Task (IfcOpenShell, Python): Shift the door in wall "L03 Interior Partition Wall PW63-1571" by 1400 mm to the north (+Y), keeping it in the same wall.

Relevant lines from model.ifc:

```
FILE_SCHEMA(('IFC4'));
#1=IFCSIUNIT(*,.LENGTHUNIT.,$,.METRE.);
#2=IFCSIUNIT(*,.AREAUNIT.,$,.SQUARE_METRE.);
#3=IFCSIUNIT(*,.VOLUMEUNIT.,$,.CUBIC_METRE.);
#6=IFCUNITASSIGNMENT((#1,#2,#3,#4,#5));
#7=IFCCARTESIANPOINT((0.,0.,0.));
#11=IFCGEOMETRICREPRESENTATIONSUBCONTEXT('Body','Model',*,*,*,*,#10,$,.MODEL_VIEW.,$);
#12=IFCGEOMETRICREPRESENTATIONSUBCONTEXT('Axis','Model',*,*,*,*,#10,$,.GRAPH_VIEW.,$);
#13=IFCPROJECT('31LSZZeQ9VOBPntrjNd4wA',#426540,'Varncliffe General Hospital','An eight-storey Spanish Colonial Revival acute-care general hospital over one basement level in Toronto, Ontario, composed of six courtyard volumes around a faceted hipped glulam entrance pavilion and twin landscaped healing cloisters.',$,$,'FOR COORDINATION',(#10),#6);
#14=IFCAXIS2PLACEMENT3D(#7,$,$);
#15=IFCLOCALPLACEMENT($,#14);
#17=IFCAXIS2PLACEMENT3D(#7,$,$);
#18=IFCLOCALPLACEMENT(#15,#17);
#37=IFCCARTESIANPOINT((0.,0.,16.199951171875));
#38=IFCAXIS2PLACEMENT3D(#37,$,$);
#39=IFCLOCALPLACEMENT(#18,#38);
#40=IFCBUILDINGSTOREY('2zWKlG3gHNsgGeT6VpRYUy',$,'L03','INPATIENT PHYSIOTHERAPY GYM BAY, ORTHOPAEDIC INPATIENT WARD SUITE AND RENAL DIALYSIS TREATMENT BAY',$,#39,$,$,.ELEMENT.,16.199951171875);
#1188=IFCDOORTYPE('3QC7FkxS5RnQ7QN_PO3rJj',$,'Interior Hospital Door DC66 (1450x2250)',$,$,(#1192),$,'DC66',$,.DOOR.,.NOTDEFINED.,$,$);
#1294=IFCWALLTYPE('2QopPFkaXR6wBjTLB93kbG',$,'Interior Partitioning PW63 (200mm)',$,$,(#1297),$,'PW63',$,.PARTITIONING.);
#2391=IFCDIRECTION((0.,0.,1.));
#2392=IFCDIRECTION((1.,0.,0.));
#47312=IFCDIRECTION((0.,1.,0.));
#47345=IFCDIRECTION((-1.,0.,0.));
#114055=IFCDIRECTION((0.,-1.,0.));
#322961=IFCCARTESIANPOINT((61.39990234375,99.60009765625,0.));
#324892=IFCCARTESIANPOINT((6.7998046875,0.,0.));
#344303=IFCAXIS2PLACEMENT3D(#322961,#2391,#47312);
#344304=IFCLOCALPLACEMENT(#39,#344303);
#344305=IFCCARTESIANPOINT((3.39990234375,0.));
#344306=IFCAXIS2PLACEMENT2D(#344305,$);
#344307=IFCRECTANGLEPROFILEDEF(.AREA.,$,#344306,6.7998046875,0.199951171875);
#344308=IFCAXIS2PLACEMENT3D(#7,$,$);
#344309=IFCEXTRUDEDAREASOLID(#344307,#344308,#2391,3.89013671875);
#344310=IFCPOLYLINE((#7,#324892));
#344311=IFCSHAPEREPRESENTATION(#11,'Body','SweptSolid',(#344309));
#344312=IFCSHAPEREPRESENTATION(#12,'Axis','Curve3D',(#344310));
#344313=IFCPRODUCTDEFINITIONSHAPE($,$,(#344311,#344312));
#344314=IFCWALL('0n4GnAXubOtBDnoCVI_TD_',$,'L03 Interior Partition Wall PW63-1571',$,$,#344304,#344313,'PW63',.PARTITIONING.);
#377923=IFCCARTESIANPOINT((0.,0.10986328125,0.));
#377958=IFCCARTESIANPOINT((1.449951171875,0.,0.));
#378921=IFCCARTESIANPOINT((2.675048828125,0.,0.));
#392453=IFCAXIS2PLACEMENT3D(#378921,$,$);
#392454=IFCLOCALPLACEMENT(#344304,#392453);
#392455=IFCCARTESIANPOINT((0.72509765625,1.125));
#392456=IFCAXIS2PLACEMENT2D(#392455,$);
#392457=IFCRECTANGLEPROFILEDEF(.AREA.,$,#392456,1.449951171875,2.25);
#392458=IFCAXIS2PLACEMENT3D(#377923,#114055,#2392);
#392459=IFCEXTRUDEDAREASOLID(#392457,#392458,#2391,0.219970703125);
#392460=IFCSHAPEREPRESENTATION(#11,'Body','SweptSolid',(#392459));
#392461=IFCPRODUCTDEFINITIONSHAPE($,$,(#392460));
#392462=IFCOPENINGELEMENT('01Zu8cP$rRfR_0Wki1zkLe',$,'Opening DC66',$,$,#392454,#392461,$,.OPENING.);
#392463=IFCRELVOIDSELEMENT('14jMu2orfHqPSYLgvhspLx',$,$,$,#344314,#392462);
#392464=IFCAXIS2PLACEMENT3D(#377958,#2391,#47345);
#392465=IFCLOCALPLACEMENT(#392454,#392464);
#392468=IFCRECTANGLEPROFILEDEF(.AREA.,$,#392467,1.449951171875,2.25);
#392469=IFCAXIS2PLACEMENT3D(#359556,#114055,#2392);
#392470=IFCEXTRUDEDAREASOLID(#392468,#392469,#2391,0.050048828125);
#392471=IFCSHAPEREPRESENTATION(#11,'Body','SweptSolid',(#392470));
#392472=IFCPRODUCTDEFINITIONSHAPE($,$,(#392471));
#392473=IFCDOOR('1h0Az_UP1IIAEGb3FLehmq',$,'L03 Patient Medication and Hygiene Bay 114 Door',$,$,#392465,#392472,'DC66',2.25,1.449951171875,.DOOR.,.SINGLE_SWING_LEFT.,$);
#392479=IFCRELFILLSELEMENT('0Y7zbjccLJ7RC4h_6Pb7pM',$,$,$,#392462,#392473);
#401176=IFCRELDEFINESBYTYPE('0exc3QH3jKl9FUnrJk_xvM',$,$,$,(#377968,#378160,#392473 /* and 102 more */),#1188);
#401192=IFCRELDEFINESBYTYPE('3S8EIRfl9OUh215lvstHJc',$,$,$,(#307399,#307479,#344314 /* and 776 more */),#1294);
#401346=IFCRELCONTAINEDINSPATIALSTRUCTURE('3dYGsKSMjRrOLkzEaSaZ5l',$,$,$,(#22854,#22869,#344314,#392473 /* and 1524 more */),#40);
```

```python
import ifcopenshell
import ifcopenshell.api.geometry
import ifcopenshell.util.placement
import ifcopenshell.util.unit

model = ifcopenshell.open("model.ifc")
unit_scale = ifcopenshell.util.unit.calculate_unit_scale(model)

door = model.by_guid("1h0Az_UP1IIAEGb3FLehmq")
opening = door.FillsVoids[0].RelatingOpeningElement
wall = opening.VoidsElements[0].RelatingBuildingElement

wall_matrix = ifcopenshell.util.placement.get_local_placement(wall.ObjectPlacement)
shift = wall_matrix[:3, 0] * 1.4 / unit_scale
before = ifcopenshell.util.placement.get_local_placement(door.ObjectPlacement)[:3, 3].copy()

# The door is placed relative to its opening, so it follows when the opening moves.
matrix = ifcopenshell.util.placement.get_local_placement(opening.ObjectPlacement)
matrix[:3, 3] += shift
ifcopenshell.api.geometry.edit_object_placement(
    model, product=opening, matrix=matrix, is_si=False, should_transform_children=True
)

after = ifcopenshell.util.placement.get_local_placement(door.ObjectPlacement)[:3, 3]
print("door moved by", (after - before).round(3) + 0.0)

model.write("model_v2.ifc")
```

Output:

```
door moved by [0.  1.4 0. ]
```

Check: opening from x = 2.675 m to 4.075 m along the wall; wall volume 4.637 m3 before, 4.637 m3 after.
